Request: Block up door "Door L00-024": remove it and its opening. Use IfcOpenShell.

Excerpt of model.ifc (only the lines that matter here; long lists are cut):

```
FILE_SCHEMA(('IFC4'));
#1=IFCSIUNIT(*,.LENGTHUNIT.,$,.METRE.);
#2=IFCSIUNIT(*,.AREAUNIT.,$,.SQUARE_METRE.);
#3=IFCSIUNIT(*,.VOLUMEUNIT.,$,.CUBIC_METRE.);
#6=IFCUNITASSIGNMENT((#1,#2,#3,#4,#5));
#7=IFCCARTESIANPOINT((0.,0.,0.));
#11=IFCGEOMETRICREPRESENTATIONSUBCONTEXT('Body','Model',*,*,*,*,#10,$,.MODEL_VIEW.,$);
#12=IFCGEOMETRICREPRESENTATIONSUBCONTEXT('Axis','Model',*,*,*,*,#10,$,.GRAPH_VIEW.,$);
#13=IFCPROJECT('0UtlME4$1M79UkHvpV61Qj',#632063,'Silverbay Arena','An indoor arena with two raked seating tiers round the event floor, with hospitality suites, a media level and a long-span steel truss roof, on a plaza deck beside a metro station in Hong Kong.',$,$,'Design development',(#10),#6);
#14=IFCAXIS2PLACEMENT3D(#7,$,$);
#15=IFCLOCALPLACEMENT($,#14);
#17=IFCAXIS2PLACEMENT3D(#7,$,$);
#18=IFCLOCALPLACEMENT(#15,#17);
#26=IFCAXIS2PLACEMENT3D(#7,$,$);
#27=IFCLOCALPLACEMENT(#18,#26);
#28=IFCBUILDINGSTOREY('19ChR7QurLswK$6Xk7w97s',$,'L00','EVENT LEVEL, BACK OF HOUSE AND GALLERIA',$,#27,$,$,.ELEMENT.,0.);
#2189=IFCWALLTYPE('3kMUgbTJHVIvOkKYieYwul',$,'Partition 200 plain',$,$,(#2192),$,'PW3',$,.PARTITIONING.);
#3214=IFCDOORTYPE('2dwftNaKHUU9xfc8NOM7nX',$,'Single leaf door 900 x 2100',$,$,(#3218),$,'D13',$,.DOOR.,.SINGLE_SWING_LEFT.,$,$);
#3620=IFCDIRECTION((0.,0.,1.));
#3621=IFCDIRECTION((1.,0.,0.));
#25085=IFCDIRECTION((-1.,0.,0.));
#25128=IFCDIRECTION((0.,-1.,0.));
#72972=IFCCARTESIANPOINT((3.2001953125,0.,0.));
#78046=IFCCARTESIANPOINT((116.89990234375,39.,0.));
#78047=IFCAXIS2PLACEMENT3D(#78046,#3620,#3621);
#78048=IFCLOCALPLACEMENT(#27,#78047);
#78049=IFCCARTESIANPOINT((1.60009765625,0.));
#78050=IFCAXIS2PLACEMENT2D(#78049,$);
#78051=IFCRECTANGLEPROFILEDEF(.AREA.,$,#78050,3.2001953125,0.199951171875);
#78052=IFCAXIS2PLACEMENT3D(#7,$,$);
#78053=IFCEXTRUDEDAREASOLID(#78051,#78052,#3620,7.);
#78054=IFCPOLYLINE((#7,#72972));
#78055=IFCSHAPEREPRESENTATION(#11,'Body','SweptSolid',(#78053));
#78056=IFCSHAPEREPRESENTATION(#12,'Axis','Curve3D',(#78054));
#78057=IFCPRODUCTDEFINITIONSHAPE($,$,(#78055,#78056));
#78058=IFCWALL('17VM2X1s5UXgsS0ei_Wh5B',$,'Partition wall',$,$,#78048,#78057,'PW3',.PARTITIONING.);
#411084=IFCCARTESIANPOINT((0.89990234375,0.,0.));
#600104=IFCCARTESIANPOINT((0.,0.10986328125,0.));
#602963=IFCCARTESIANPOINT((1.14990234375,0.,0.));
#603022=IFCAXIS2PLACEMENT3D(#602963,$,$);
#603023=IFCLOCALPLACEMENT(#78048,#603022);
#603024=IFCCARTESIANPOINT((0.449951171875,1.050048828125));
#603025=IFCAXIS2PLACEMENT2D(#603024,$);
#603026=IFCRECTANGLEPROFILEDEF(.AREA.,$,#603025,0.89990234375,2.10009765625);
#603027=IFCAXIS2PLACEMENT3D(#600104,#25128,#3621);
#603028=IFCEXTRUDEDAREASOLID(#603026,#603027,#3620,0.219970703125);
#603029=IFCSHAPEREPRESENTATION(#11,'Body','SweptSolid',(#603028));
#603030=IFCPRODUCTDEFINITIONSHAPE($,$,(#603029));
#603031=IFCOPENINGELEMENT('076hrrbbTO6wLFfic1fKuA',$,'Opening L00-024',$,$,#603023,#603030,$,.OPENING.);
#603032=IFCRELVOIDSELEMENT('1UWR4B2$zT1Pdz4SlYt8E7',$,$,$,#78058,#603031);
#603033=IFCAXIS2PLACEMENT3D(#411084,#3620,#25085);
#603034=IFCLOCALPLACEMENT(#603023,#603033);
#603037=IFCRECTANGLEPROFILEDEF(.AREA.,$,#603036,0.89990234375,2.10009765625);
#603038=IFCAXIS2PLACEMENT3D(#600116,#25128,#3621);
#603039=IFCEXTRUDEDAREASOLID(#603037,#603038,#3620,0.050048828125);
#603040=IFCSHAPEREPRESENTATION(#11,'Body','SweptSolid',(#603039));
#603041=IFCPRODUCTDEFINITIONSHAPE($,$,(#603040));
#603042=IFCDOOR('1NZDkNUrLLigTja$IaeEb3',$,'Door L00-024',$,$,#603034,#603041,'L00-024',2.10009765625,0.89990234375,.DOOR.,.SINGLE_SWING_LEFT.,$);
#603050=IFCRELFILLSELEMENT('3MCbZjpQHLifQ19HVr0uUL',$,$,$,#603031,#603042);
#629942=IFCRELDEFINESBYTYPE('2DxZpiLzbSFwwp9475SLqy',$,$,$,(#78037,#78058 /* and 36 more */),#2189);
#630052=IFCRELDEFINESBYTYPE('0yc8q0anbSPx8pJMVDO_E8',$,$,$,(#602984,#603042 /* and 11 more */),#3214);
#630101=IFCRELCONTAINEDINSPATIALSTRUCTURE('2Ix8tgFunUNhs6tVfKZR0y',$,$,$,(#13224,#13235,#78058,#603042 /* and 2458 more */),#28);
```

```python
import ifcopenshell
import ifcopenshell.api.feature
import ifcopenshell.api.root
import ifcopenshell.geom
import ifcopenshell.util.shape

model = ifcopenshell.open("model.ifc")
settings = ifcopenshell.geom.settings()


def volume(element):
    """Net volume in cubic metres, openings subtracted."""
    shape = ifcopenshell.geom.create_shape(settings, element)
    return ifcopenshell.util.shape.get_volume(shape.geometry)


door = model.by_guid("1NZDkNUrLLigTja$IaeEb3")
opening = door.FillsVoids[0].RelatingOpeningElement
wall = opening.VoidsElements[0].RelatingBuildingElement
before = volume(wall)

ifcopenshell.api.root.remove_product(model, product=door)
ifcopenshell.api.feature.remove_feature(model, feature=opening)

after = volume(wall)

print(f"wall volume {before:.3f} -> {after:.3f} m3")

model.write("model_edited.ifc")
```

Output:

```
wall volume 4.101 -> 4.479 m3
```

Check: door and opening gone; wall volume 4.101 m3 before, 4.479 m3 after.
